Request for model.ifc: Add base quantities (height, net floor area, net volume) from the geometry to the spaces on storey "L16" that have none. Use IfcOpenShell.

First a look at what the model holds.

```python
import ifcopenshell
import ifcopenshell.util.element
import ifcopenshell.util.unit

model = ifcopenshell.open("model.ifc")
print(model.schema)
for unit_type in ("LENGTHUNIT", "AREAUNIT", "VOLUMEUNIT"):
    print(unit_type, ifcopenshell.util.unit.calculate_unit_scale(model, unit_type))
storey = next(s for s in model.by_type("IfcBuildingStorey") if s.Name == "L16")
spaces = [e for e in ifcopenshell.util.element.get_decomposition(storey) if e.is_a("IfcSpace")]
for e in sorted(spaces, key=lambda e: e.id()):
    print(e.id(), e.is_a(), e.Name, list(ifcopenshell.util.element.get_psets(e, qtos_only=True)), sep=" | ")
```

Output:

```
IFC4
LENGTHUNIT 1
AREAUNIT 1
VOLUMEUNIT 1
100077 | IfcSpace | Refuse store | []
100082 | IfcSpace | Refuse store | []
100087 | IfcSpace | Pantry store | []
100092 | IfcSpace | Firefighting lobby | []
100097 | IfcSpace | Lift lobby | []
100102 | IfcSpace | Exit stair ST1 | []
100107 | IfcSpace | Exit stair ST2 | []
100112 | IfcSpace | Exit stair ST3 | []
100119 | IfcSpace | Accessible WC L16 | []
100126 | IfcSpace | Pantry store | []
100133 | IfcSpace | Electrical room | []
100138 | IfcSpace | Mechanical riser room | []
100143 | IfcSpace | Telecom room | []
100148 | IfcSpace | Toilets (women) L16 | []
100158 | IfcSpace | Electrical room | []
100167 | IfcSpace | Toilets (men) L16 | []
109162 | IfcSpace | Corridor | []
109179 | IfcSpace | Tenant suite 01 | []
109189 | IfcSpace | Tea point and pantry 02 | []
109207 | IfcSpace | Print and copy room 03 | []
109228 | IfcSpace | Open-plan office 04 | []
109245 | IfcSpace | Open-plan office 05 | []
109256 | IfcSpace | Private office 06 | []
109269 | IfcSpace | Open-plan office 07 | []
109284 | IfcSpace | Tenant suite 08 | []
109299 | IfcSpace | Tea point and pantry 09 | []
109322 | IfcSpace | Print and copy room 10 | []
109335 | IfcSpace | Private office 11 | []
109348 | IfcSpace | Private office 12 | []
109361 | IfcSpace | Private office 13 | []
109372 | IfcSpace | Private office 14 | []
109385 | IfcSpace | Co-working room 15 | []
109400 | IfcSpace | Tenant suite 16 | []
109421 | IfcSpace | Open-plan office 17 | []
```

```python
import ifcopenshell
import ifcopenshell.api.pset
import ifcopenshell.geom
import ifcopenshell.util.element
import ifcopenshell.util.shape
import ifcopenshell.util.unit

model = ifcopenshell.open("model.ifc")
unit_scale = ifcopenshell.util.unit.calculate_unit_scale(model)
area_scale = ifcopenshell.util.unit.calculate_unit_scale(model, "AREAUNIT")
volume_scale = ifcopenshell.util.unit.calculate_unit_scale(model, "VOLUMEUNIT")
settings = ifcopenshell.geom.settings()

storey = next(s for s in model.by_type("IfcBuildingStorey") if s.Name == "L16")
spaces = [e for e in ifcopenshell.util.element.get_decomposition(storey) if e.is_a("IfcSpace")]

for e in sorted(spaces, key=lambda e: e.id()):
    if ifcopenshell.util.element.get_psets(e, qtos_only=True, should_inherit=False):
        continue
    # Geometry comes back in metres, in the element's own axes.
    shape = ifcopenshell.geom.create_shape(settings, e)
    values = {
        "Height": ifcopenshell.util.shape.get_z(shape.geometry) / unit_scale,
        "NetFloorArea": ifcopenshell.util.shape.get_footprint_area(shape.geometry) / area_scale,
        "NetVolume": ifcopenshell.util.shape.get_volume(shape.geometry) / volume_scale,
    }
    qto = ifcopenshell.api.pset.add_qto(model, product=e, name="Qto_SpaceBaseQuantities")
    ifcopenshell.api.pset.edit_qto(model, qto=qto, properties=values)
    print(e.id(), {k: round(v, 3) for k, v in values.items()})

model.write("model_rev.ifc")
```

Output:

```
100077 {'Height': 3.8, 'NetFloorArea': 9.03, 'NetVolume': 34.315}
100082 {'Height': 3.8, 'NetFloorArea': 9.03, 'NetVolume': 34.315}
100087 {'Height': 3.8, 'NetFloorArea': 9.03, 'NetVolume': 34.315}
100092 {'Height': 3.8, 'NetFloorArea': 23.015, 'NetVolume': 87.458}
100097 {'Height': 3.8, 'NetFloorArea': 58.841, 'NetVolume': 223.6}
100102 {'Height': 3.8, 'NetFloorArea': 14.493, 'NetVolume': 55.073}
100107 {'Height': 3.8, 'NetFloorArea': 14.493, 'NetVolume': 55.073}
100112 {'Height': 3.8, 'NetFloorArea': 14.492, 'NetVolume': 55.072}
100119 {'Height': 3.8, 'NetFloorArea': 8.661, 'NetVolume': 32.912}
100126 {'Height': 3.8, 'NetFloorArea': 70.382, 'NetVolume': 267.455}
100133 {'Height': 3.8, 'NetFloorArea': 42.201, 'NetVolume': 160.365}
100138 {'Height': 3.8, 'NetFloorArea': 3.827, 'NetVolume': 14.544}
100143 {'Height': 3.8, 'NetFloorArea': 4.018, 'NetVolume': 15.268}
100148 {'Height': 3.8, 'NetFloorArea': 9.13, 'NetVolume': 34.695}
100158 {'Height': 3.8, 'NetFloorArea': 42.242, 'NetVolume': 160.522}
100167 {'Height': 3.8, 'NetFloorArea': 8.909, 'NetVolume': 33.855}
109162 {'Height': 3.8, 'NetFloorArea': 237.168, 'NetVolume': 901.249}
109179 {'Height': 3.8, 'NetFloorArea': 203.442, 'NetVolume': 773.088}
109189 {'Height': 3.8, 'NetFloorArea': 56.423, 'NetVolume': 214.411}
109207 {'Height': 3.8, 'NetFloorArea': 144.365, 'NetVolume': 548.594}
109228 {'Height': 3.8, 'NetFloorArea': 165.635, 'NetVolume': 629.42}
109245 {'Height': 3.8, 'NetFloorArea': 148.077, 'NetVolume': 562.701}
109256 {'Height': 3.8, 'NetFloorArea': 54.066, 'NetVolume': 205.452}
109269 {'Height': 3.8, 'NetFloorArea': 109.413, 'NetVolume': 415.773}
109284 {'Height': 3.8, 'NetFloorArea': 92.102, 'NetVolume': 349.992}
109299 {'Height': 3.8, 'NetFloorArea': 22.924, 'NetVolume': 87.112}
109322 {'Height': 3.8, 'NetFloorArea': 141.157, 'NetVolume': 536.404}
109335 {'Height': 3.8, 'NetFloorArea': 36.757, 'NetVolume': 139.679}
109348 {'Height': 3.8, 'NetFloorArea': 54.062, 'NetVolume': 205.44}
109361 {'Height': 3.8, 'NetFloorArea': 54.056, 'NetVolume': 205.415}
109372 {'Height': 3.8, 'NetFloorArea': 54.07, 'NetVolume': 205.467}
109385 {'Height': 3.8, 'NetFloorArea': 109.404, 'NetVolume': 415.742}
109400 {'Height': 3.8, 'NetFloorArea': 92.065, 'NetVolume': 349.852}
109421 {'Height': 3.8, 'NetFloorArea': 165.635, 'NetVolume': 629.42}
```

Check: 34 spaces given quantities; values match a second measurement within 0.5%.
